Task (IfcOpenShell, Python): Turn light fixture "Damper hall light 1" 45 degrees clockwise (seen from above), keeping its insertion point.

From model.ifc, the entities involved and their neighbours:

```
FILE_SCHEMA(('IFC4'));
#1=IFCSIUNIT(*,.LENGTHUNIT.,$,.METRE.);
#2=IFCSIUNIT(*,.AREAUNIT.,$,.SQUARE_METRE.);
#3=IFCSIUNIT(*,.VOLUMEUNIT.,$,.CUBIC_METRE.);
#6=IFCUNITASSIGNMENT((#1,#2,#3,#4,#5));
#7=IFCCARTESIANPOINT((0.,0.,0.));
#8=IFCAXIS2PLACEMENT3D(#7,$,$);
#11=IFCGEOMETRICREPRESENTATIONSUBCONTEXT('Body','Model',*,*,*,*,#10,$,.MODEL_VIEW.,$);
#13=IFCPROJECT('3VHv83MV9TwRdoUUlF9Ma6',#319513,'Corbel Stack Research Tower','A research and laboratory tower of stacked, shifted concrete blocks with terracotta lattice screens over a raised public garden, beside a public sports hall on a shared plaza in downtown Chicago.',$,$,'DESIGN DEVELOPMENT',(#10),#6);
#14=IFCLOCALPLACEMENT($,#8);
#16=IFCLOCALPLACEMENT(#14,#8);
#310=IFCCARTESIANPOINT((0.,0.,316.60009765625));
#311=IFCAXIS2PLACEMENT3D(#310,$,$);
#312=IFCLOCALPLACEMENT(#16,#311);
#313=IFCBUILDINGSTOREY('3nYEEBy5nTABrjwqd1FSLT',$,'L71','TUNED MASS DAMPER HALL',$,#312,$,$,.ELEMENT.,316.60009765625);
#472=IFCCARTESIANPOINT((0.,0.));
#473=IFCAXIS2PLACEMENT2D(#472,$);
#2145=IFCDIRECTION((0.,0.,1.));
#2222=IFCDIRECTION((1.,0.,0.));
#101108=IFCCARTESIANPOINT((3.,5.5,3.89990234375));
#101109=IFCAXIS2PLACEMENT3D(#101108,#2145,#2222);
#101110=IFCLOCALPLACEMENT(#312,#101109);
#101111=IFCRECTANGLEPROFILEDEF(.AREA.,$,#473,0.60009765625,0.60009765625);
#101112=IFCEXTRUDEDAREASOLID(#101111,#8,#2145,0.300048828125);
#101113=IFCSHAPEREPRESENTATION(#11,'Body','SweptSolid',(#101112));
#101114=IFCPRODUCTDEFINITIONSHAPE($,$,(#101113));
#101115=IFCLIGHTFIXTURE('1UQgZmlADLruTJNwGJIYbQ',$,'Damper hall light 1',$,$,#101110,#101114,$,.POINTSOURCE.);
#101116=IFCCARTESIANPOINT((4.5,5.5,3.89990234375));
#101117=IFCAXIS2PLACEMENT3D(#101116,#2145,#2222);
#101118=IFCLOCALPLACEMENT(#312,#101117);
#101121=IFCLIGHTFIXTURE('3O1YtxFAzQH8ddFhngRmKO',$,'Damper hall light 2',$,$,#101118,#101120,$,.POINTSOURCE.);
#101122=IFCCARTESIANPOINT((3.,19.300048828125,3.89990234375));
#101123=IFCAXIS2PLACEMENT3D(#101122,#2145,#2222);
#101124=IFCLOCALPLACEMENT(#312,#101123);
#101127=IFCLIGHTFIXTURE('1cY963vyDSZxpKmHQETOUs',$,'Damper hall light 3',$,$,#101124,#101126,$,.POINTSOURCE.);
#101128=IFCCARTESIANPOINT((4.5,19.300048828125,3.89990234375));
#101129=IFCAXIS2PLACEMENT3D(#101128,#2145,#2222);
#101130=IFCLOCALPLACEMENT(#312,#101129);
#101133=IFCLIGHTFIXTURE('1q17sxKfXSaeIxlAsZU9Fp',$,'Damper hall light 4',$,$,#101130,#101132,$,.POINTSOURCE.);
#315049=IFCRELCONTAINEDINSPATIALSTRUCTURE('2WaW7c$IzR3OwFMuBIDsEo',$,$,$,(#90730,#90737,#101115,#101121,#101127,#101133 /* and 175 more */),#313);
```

```python
import ifcopenshell
import ifcopenshell.api.geometry
import ifcopenshell.util.placement

model = ifcopenshell.open("model.ifc")

item = model.by_guid("1UQgZmlADLruTJNwGJIYbQ")
matrix = ifcopenshell.util.placement.get_local_placement(item.ObjectPlacement)
matrix = matrix @ ifcopenshell.util.placement.rotation(-45, "Z")
ifcopenshell.api.geometry.edit_object_placement(model, product=item, matrix=matrix, is_si=False)

print(ifcopenshell.util.placement.get_local_placement(item.ObjectPlacement).round(3) + 0.0)

model.write("model_edited.ifc")
```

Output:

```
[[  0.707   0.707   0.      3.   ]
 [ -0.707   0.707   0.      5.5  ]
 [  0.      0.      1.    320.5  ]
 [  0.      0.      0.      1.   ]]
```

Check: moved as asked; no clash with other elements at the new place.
